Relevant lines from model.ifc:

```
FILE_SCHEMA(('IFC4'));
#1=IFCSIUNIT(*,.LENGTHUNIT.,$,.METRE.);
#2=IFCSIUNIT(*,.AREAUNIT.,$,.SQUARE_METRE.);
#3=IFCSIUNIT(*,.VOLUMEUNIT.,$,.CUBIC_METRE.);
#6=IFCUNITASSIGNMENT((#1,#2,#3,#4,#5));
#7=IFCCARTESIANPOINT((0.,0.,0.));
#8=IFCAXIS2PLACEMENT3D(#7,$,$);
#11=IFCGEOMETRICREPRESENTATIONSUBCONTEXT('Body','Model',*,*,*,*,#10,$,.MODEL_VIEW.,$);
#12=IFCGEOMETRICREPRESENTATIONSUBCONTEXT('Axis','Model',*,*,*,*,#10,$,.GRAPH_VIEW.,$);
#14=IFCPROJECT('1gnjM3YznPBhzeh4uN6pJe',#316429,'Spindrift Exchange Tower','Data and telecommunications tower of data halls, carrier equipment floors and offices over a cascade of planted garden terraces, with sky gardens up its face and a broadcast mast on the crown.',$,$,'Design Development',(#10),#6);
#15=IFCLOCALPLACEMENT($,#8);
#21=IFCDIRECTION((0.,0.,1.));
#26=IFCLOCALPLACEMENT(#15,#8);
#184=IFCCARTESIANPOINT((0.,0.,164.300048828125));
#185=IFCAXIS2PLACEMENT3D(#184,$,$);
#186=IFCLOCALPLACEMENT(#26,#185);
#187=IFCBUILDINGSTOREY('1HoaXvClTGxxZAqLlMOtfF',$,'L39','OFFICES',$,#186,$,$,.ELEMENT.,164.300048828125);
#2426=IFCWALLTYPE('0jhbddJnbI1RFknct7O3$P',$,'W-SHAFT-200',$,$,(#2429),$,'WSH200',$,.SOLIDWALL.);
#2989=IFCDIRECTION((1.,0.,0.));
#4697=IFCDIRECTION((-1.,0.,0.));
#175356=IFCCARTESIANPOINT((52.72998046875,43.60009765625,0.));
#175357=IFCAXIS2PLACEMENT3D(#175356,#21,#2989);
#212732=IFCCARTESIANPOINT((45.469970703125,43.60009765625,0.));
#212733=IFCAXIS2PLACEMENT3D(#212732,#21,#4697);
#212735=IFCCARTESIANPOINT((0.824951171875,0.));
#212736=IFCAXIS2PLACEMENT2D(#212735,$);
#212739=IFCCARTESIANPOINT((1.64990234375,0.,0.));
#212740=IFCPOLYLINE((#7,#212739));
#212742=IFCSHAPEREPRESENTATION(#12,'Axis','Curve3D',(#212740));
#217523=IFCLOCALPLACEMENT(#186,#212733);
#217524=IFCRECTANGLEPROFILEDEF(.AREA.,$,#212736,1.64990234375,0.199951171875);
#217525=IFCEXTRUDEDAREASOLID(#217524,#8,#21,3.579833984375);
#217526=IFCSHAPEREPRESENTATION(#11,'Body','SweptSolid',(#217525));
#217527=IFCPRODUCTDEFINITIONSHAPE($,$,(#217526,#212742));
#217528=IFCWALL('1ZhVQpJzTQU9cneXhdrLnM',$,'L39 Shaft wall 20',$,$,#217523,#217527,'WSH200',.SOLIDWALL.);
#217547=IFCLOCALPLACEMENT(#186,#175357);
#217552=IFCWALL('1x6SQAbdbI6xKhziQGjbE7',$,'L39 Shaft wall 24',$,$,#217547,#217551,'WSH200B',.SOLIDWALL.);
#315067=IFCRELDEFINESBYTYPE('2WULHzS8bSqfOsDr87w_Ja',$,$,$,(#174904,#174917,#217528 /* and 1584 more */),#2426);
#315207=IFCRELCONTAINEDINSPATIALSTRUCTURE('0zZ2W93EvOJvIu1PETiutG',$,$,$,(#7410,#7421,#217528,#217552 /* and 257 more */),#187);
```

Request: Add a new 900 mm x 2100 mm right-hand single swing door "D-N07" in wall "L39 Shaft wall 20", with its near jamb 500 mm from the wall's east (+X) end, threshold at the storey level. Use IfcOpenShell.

```python
import numpy as np
import ifcopenshell
import ifcopenshell.api.feature
import ifcopenshell.api.geometry
import ifcopenshell.api.root
import ifcopenshell.api.spatial
import ifcopenshell.geom
import ifcopenshell.util.element
import ifcopenshell.util.placement
import ifcopenshell.util.representation
import ifcopenshell.util.shape
import ifcopenshell.util.unit

model = ifcopenshell.open("model.ifc")
unit_scale = ifcopenshell.util.unit.calculate_unit_scale(model)
settings = ifcopenshell.geom.settings()


def volume(element):
    """Net volume in cubic metres, openings subtracted."""
    shape = ifcopenshell.geom.create_shape(settings, element)
    return ifcopenshell.util.shape.get_volume(shape.geometry)


wall = model.by_id(217528)
storey = ifcopenshell.util.element.get_container(wall, ifc_class="IfcBuildingStorey")
context = ifcopenshell.util.representation.get_context(model, "Model", "Body", "MODEL_VIEW")
before = volume(wall)

width, height, from_end, sill = 0.9, 2.1, 0.5, 0.0  # metres

# The wall runs along its own X axis, and the end named is its -X end.
wall_shape = ifcopenshell.geom.create_shape(settings, wall)
x, y, z = ifcopenshell.util.shape.get_vertices(wall_shape.geometry).T
start = x.min() + from_end
face, thickness = float(y.min()), float(y.max() - y.min())
wall_matrix = ifcopenshell.util.placement.get_local_placement(wall.ObjectPlacement)
level = ifcopenshell.util.placement.get_local_placement(storey.ObjectPlacement)[2, 3]


def in_wall(x, y):
    """Placement at x, y metres in the wall's axes, at sill height."""
    matrix = wall_matrix.copy()
    matrix[:, 3] = wall_matrix @ np.array([x / unit_scale, y / unit_scale, 0.0, 1.0])
    matrix[2, 3] = level + sill / unit_scale
    return matrix


# Opening: a box that overshoots both wall faces by 50 mm.
opening = ifcopenshell.api.root.create_entity(model, ifc_class="IfcOpeningElement", predefined_type="OPENING")
box = ifcopenshell.api.geometry.add_wall_representation(
    model, context=context, length=width, height=height, thickness=thickness + 0.1
)
ifcopenshell.api.geometry.assign_representation(model, product=opening, representation=box)
ifcopenshell.api.geometry.edit_object_placement(model, product=opening, matrix=in_wall(start, face - 0.05), is_si=False)
ifcopenshell.api.feature.add_feature(model, feature=opening, element=wall)

door = ifcopenshell.api.root.create_entity(model, ifc_class="IfcDoor", name="D-N07", predefined_type="DOOR")
door.OverallWidth, door.OverallHeight = width / unit_scale, height / unit_scale
door.OperationType = "SINGLE_SWING_RIGHT"
body = ifcopenshell.api.geometry.add_door_representation(
    model,
    context=context,
    overall_width=door.OverallWidth,
    overall_height=door.OverallHeight,
    operation_type="SINGLE_SWING_RIGHT",
    lining_properties={"LiningDepth": thickness / unit_scale, "ThresholdDepth": thickness / unit_scale},
)
ifcopenshell.api.geometry.assign_representation(model, product=door, representation=body)
ifcopenshell.api.spatial.assign_container(model, products=[door], relating_structure=storey)
ifcopenshell.api.feature.add_filling(model, opening=opening, element=door)

# The lining spans the wall, so the door starts at the wall face.
ifcopenshell.api.geometry.edit_object_placement(model, product=door, matrix=in_wall(start, face), is_si=False)

after = volume(wall)

print(f"wall volume {before:.3f} -> {after:.3f} m3")

model.write("model-out.ifc")
```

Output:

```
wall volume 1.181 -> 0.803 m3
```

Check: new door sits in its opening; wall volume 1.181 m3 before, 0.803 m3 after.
